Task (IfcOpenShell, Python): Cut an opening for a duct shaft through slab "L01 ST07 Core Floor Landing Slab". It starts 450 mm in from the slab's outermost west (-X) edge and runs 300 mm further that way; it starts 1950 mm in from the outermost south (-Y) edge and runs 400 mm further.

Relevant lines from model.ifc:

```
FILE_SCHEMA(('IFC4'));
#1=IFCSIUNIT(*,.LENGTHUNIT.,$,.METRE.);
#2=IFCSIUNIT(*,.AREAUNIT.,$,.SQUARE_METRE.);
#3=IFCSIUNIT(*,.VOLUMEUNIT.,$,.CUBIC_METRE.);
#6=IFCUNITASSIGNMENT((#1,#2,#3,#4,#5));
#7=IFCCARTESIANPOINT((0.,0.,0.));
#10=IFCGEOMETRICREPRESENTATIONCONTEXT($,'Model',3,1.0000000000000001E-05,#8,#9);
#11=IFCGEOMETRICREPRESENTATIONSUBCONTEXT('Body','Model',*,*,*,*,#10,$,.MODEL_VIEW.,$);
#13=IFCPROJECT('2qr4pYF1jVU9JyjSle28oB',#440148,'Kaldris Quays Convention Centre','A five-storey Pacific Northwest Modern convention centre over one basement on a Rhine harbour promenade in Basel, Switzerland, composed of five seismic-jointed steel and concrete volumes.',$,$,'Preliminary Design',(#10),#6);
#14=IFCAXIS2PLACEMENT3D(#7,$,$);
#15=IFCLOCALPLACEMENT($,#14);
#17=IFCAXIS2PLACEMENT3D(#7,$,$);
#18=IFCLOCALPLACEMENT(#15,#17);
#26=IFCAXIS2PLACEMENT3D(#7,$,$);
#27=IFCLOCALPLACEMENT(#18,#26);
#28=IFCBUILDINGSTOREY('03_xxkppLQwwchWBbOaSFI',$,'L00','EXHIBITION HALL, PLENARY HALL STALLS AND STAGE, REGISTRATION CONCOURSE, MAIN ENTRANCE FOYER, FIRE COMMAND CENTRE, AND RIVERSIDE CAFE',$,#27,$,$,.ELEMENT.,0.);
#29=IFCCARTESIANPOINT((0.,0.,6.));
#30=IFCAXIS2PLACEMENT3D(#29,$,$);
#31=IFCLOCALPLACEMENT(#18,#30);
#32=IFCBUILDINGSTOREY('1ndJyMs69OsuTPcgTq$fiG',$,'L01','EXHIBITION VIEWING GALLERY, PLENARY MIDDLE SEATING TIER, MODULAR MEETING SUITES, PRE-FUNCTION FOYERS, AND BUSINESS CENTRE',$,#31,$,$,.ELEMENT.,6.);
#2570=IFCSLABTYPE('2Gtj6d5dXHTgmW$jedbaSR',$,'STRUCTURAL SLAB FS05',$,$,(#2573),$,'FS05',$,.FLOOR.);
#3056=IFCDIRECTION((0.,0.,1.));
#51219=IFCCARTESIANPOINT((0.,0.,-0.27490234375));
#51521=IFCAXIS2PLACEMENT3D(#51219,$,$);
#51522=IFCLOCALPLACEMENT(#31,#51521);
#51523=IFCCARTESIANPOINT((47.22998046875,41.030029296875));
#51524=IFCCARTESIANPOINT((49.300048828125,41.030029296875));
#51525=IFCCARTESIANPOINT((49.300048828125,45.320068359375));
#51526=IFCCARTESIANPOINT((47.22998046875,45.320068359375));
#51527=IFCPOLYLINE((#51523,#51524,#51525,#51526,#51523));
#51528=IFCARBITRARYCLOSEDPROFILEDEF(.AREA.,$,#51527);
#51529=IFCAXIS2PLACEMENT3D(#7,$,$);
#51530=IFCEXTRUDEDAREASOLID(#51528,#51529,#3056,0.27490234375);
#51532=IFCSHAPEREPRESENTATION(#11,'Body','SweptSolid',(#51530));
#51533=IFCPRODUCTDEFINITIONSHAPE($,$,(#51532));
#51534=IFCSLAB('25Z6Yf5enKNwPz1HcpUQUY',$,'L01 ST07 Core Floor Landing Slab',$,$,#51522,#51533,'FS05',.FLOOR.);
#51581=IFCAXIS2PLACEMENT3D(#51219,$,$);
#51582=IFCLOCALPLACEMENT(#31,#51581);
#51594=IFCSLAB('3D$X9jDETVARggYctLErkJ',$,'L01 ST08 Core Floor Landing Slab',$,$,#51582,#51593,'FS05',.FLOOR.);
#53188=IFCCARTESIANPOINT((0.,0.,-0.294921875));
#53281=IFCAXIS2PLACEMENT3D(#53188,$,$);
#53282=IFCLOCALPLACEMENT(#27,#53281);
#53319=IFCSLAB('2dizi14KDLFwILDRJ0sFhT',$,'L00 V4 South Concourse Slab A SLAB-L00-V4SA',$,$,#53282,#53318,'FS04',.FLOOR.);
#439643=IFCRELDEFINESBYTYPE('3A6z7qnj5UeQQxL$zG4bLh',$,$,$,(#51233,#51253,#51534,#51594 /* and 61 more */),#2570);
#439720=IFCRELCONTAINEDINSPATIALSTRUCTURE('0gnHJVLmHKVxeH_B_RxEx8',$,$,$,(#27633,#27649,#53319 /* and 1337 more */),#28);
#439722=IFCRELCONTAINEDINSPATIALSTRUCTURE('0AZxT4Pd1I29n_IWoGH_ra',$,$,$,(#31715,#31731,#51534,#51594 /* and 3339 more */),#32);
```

```python
import numpy as np
import ifcopenshell
import ifcopenshell.api.feature
import ifcopenshell.api.geometry
import ifcopenshell.api.root
import ifcopenshell.geom
import ifcopenshell.util.placement
import ifcopenshell.util.representation
import ifcopenshell.util.shape
import ifcopenshell.util.unit

model = ifcopenshell.open("model.ifc")
unit_scale = ifcopenshell.util.unit.calculate_unit_scale(model)
settings = ifcopenshell.geom.settings()


def volume(element):
    """Net volume in cubic metres, openings subtracted."""
    shape = ifcopenshell.geom.create_shape(settings, element)
    return ifcopenshell.util.shape.get_volume(shape.geometry)


slab = model.by_guid("25Z6Yf5enKNwPz1HcpUQUY")
before = volume(slab)

# Extent in the slab's own axes, in metres. The edges named are its -X and -Y sides.
slab_shape = ifcopenshell.geom.create_shape(settings, slab)
vertices = ifcopenshell.util.shape.get_vertices(slab_shape.geometry)
x_min, y_min, bottom = vertices.min(axis=0)
top = vertices[:, 2].max()

opening = ifcopenshell.api.root.create_entity(model, ifc_class="IfcOpeningElement", name="Duct shaft opening", predefined_type="OPENING")
context = ifcopenshell.util.representation.get_context(model, "Model", "Body", "MODEL_VIEW")
width, depth = 0.3, 0.4
outline = [(0.0, 0.0), (width, 0.0), (width, depth), (0.0, depth), (0.0, 0.0)]
# Overshoot both faces by 50 mm so the cut is clean.
shape = ifcopenshell.api.geometry.add_slab_representation(
    model, context=context, depth=top - bottom + 0.1, polyline=outline
)
ifcopenshell.api.geometry.assign_representation(model, product=opening, representation=shape)

matrix = ifcopenshell.util.placement.get_local_placement(slab.ObjectPlacement)
matrix[:, 3] = matrix @ np.append(np.array([x_min + 0.45, y_min + 1.95, bottom - 0.05]) / unit_scale, 1.0)
ifcopenshell.api.geometry.edit_object_placement(model, product=opening, matrix=matrix, is_si=False)
ifcopenshell.api.feature.add_feature(model, feature=opening, element=slab)

after = volume(slab)

print(f"slab volume {before:.3f} -> {after:.3f} m3")

model.write("model_updated.ifc")
```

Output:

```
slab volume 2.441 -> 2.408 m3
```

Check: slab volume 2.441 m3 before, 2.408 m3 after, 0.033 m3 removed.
